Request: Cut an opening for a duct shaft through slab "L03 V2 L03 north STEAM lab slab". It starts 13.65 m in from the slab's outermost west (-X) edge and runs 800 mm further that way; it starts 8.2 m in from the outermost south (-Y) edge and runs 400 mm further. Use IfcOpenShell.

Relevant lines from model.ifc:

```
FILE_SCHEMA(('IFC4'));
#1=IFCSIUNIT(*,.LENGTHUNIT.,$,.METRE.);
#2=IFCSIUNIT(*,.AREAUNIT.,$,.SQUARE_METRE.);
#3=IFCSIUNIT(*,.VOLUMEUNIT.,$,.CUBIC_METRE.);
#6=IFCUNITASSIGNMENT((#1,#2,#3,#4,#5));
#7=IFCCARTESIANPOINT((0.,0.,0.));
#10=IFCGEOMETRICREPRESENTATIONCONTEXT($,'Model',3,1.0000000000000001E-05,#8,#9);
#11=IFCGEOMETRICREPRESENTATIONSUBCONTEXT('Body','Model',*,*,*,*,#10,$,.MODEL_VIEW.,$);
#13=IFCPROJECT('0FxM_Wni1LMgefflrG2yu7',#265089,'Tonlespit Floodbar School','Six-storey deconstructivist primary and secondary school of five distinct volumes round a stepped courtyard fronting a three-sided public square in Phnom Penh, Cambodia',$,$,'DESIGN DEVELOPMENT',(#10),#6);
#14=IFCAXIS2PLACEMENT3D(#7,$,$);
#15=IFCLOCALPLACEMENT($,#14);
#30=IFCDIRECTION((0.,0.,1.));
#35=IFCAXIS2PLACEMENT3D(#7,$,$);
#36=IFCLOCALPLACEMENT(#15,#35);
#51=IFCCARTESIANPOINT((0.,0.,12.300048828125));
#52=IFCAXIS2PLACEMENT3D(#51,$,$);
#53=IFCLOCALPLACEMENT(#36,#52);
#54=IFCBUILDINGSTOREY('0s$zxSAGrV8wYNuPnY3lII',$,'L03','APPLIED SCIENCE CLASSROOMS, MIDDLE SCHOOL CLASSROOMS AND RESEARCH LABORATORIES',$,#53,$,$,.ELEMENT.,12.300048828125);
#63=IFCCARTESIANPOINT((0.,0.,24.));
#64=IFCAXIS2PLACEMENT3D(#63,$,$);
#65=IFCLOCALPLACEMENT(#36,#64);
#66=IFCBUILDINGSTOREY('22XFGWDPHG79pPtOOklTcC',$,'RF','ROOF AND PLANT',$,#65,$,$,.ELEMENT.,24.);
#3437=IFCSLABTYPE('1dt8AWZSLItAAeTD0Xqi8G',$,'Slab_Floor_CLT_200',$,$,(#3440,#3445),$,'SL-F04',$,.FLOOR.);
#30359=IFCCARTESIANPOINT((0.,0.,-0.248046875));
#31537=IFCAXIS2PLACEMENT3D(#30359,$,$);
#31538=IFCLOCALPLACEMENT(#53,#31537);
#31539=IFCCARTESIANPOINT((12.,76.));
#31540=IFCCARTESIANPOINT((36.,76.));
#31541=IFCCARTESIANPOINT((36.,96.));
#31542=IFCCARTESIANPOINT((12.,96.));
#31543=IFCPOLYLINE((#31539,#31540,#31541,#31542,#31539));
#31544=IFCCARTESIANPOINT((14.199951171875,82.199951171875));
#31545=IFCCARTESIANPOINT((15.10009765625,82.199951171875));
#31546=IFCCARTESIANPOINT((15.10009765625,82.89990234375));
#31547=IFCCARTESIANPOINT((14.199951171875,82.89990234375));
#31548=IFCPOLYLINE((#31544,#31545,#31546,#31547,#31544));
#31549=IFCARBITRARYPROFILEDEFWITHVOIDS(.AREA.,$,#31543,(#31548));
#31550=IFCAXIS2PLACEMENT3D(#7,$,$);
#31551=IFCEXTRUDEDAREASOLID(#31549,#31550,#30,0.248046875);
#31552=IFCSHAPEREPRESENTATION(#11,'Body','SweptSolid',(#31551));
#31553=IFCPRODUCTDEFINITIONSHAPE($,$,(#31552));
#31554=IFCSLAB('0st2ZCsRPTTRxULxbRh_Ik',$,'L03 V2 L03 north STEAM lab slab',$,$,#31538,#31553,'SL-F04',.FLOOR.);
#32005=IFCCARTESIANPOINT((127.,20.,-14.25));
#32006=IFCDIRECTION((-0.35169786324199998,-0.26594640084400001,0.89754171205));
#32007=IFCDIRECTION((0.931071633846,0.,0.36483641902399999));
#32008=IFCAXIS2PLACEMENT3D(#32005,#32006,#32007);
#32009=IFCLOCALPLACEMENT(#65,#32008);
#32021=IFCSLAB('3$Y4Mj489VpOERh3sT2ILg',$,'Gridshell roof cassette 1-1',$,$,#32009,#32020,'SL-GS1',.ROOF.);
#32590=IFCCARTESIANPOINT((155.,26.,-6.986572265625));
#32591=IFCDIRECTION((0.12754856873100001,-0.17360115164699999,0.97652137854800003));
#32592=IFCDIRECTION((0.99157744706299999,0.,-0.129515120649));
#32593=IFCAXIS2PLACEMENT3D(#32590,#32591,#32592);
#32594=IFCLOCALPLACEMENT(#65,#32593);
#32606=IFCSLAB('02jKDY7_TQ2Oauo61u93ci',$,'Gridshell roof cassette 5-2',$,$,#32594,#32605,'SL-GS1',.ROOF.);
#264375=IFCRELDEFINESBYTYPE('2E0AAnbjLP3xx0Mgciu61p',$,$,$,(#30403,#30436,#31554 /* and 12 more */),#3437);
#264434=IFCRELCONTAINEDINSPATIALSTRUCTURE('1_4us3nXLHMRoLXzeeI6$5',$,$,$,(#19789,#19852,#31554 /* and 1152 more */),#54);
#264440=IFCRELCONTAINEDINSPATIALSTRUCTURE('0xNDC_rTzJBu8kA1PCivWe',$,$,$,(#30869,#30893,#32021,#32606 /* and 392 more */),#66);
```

```python
import numpy as np
import ifcopenshell
import ifcopenshell.api.feature
import ifcopenshell.api.geometry
import ifcopenshell.api.root
import ifcopenshell.geom
import ifcopenshell.util.placement
import ifcopenshell.util.representation
import ifcopenshell.util.shape
import ifcopenshell.util.unit

model = ifcopenshell.open("model.ifc")
unit_scale = ifcopenshell.util.unit.calculate_unit_scale(model)
settings = ifcopenshell.geom.settings()


def volume(element):
    """Net volume in cubic metres, openings subtracted."""
    shape = ifcopenshell.geom.create_shape(settings, element)
    return ifcopenshell.util.shape.get_volume(shape.geometry)


slab = model.by_guid("0st2ZCsRPTTRxULxbRh_Ik")
before = volume(slab)

# Extent in the slab's own axes, in metres. The edges named are its -X and -Y sides.
slab_shape = ifcopenshell.geom.create_shape(settings, slab)
vertices = ifcopenshell.util.shape.get_vertices(slab_shape.geometry)
x_min, y_min, bottom = vertices.min(axis=0)
top = vertices[:, 2].max()

opening = ifcopenshell.api.root.create_entity(model, ifc_class="IfcOpeningElement", name="Duct shaft opening", predefined_type="OPENING")
context = ifcopenshell.util.representation.get_context(model, "Model", "Body", "MODEL_VIEW")
width, depth = 0.8, 0.4
outline = [(0.0, 0.0), (width, 0.0), (width, depth), (0.0, depth), (0.0, 0.0)]
# Overshoot both faces by 50 mm so the cut is clean.
shape = ifcopenshell.api.geometry.add_slab_representation(
    model, context=context, depth=top - bottom + 0.1, polyline=outline
)
ifcopenshell.api.geometry.assign_representation(model, product=opening, representation=shape)

matrix = ifcopenshell.util.placement.get_local_placement(slab.ObjectPlacement)
matrix[:, 3] = matrix @ np.append(np.array([x_min + 13.65, y_min + 8.2, bottom - 0.05]) / unit_scale, 1.0)
ifcopenshell.api.geometry.edit_object_placement(model, product=opening, matrix=matrix, is_si=False)
ifcopenshell.api.feature.add_feature(model, feature=opening, element=slab)

after = volume(slab)

print(f"slab volume {before:.3f} -> {after:.3f} m3")

model.write("model_updated.ifc")
```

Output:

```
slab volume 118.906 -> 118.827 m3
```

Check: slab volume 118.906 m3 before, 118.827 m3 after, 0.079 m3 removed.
